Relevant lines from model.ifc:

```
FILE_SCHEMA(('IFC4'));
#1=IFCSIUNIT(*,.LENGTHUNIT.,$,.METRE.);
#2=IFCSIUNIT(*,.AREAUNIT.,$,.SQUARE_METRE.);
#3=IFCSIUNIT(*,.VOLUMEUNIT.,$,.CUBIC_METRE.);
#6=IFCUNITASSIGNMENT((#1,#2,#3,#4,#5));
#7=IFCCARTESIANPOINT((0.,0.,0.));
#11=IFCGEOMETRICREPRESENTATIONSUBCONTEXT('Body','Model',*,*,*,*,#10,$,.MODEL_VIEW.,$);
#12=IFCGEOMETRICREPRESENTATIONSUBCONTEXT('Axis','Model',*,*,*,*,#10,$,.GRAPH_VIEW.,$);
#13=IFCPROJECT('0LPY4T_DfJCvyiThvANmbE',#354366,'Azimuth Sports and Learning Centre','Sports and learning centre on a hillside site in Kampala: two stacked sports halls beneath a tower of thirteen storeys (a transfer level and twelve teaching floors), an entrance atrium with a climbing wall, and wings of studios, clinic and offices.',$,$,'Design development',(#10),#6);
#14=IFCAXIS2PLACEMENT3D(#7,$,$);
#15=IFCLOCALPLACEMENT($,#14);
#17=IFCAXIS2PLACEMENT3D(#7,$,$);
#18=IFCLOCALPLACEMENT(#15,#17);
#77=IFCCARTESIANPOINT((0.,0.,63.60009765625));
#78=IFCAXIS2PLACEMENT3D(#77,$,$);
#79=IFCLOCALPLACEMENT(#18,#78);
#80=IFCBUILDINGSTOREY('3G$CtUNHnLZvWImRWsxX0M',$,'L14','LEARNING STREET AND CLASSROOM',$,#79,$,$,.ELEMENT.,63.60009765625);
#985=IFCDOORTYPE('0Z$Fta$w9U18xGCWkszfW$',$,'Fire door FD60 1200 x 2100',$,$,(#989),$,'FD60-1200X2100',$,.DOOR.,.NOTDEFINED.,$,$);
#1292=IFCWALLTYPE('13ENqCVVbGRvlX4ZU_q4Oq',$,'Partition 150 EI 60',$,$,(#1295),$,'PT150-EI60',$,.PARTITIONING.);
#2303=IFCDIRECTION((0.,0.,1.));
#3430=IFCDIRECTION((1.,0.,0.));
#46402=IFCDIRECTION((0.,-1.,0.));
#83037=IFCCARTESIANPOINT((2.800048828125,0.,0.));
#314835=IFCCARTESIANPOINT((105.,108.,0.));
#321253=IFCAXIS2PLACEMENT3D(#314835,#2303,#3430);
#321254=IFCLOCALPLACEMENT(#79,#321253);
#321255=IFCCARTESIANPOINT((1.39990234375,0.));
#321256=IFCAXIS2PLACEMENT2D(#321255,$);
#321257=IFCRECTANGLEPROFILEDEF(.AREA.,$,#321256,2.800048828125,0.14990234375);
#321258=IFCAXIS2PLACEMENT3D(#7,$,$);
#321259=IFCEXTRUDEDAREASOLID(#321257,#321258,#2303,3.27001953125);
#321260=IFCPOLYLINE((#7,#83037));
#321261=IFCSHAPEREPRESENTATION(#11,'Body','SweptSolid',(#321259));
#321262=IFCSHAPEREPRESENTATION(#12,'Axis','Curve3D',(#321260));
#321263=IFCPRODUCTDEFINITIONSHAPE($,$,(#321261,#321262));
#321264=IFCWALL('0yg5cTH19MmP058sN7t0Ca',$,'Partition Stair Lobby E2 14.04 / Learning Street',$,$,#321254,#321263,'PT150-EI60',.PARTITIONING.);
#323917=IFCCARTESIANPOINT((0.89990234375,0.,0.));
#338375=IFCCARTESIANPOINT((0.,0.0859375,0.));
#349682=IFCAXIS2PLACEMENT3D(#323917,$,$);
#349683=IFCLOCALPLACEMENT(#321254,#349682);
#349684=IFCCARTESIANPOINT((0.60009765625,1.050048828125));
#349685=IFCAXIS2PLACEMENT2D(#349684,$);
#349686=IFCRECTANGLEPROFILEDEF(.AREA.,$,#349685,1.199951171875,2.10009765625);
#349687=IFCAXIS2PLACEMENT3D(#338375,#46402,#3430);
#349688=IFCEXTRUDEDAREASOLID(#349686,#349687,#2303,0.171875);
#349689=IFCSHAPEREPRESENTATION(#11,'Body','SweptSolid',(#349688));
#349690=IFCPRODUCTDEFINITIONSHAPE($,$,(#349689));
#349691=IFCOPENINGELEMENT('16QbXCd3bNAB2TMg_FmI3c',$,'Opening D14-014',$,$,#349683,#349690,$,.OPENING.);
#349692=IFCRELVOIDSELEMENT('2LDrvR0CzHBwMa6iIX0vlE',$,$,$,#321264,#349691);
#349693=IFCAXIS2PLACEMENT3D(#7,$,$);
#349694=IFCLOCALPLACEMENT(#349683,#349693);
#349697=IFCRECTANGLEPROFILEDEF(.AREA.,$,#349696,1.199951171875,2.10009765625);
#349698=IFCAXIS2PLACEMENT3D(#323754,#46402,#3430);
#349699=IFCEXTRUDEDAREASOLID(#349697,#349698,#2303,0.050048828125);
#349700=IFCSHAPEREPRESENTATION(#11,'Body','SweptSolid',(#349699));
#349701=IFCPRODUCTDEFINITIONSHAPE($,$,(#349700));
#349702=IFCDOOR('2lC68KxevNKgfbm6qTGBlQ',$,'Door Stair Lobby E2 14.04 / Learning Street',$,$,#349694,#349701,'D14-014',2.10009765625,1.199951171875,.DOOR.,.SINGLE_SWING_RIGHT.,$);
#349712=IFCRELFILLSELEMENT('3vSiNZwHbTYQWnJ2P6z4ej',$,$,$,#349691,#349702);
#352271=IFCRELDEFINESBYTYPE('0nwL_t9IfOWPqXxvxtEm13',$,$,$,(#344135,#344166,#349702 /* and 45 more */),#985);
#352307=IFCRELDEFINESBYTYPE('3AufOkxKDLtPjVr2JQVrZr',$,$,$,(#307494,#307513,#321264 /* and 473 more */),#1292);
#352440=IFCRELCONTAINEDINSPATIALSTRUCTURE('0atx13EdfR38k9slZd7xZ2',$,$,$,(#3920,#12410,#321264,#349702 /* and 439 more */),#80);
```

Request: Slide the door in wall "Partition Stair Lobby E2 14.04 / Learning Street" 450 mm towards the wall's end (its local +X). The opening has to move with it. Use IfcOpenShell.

```python
import ifcopenshell
import ifcopenshell.api.geometry
import ifcopenshell.util.placement

model = ifcopenshell.open("model.ifc")

door = model.by_guid("2lC68KxevNKgfbm6qTGBlQ")
opening = door.FillsVoids[0].RelatingOpeningElement
wall = opening.VoidsElements[0].RelatingBuildingElement

wall_matrix = ifcopenshell.util.placement.get_local_placement(wall.ObjectPlacement)
shift = wall_matrix[:3, 0] * 0.45
before = ifcopenshell.util.placement.get_local_placement(door.ObjectPlacement)[:3, 3].copy()

# The door is placed relative to its opening, so it follows when the opening moves.
matrix = ifcopenshell.util.placement.get_local_placement(opening.ObjectPlacement)
matrix[:3, 3] += shift
ifcopenshell.api.geometry.edit_object_placement(
    model, product=opening, matrix=matrix, is_si=False, should_transform_children=True
)

after = ifcopenshell.util.placement.get_local_placement(door.ObjectPlacement)[:3, 3]
print("door moved by", (after - before).round(3) + 0.0)

model.write("model_rev.ifc")
```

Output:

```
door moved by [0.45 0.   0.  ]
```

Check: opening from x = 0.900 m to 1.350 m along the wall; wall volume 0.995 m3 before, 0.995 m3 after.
